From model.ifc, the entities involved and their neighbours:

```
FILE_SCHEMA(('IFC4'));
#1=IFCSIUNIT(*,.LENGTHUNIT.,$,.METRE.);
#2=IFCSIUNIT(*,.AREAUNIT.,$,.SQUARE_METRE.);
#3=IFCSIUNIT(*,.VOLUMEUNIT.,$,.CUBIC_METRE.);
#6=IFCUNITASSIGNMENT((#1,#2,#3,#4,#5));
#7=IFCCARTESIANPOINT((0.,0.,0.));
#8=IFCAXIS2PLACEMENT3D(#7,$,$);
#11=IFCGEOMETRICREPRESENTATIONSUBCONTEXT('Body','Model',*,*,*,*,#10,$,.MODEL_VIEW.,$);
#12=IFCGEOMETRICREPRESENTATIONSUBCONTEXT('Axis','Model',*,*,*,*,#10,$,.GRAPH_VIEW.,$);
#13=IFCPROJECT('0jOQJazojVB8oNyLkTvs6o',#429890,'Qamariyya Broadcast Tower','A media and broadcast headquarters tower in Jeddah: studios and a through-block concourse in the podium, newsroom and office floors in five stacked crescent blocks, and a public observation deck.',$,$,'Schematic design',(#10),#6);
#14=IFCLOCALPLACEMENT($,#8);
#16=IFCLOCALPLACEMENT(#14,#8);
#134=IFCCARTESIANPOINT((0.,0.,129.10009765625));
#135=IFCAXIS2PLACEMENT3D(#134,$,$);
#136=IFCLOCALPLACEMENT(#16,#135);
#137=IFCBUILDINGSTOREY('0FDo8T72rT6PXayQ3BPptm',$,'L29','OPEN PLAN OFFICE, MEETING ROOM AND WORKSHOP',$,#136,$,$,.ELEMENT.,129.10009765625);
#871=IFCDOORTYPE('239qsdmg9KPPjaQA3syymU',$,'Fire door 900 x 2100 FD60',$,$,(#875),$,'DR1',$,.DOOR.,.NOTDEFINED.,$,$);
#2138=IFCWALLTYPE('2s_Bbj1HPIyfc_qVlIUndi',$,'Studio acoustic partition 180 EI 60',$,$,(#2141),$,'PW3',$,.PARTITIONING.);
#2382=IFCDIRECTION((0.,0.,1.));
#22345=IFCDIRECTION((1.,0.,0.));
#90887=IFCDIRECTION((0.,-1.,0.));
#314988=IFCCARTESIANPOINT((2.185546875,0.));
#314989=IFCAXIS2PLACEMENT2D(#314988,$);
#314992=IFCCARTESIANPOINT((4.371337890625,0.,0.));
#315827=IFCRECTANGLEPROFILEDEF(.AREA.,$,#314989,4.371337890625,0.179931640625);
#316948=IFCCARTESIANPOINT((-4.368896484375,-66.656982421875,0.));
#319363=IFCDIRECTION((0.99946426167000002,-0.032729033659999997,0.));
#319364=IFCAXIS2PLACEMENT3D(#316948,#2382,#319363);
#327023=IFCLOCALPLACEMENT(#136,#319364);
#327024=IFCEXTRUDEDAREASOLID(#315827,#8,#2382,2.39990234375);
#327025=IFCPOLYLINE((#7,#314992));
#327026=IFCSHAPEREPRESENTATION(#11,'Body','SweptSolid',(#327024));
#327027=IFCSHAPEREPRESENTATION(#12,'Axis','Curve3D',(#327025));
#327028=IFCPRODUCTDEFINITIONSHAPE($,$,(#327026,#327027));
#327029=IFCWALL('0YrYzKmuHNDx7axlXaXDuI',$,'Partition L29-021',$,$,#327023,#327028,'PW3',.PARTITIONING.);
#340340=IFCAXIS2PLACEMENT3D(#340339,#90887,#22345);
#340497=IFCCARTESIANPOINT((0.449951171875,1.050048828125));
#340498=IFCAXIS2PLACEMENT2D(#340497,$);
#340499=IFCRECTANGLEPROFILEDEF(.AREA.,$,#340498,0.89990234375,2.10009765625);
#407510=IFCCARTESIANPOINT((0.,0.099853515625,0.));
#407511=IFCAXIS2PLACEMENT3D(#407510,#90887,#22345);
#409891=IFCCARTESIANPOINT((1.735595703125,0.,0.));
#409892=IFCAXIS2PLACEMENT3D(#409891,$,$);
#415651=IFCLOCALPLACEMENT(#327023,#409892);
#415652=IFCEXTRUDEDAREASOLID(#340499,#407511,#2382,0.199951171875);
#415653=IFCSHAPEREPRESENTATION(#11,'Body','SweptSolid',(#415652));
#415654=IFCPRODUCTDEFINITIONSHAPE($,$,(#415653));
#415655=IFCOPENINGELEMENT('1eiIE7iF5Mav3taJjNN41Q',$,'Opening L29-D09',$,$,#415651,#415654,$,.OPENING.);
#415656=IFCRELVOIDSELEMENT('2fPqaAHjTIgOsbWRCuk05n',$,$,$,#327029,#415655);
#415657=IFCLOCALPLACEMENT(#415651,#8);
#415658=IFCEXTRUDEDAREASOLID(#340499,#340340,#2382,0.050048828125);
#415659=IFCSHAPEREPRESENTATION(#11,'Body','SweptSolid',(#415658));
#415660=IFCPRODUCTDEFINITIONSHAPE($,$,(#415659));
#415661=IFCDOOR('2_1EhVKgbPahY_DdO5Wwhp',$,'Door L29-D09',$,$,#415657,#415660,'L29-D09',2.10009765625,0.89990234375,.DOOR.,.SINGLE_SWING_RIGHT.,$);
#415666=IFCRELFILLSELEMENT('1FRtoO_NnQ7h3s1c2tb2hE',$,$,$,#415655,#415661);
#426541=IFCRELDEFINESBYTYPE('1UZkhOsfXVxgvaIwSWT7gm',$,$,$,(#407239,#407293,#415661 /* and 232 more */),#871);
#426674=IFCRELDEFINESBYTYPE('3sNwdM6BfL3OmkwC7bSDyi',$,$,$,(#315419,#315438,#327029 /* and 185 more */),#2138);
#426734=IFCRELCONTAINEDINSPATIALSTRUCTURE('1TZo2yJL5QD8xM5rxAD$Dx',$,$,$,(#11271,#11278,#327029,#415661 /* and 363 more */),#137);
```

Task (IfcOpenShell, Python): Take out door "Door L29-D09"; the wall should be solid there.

```python
import ifcopenshell
import ifcopenshell.api.feature
import ifcopenshell.api.root
import ifcopenshell.geom
import ifcopenshell.util.shape

model = ifcopenshell.open("model.ifc")
settings = ifcopenshell.geom.settings()


def volume(element):
    """Net volume in cubic metres, openings subtracted."""
    shape = ifcopenshell.geom.create_shape(settings, element)
    return ifcopenshell.util.shape.get_volume(shape.geometry)


door = model.by_guid("2_1EhVKgbPahY_DdO5Wwhp")
opening = door.FillsVoids[0].RelatingOpeningElement
wall = opening.VoidsElements[0].RelatingBuildingElement
before = volume(wall)

ifcopenshell.api.root.remove_product(model, product=door)
ifcopenshell.api.feature.remove_feature(model, feature=opening)

after = volume(wall)

print(f"wall volume {before:.3f} -> {after:.3f} m3")

model.write("model_v2.ifc")
```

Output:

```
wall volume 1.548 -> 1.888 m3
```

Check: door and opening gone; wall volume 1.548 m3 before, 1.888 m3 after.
